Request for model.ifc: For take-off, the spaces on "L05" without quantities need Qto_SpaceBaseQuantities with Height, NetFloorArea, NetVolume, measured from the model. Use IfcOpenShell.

First a look at what the model holds.

```python
import ifcopenshell
import ifcopenshell.util.element
import ifcopenshell.util.unit

model = ifcopenshell.open("model.ifc")
print(model.schema)
for unit_type in ("LENGTHUNIT", "AREAUNIT", "VOLUMEUNIT"):
    print(unit_type, ifcopenshell.util.unit.calculate_unit_scale(model, unit_type))
storey = next(s for s in model.by_type("IfcBuildingStorey") if s.Name == "L05")
spaces = [e for e in ifcopenshell.util.element.get_decomposition(storey) if e.is_a("IfcSpace")]
for e in sorted(spaces, key=lambda e: e.id()):
    print(e.id(), e.is_a(), e.Name, list(ifcopenshell.util.element.get_psets(e, qtos_only=True)), sep=" | ")
```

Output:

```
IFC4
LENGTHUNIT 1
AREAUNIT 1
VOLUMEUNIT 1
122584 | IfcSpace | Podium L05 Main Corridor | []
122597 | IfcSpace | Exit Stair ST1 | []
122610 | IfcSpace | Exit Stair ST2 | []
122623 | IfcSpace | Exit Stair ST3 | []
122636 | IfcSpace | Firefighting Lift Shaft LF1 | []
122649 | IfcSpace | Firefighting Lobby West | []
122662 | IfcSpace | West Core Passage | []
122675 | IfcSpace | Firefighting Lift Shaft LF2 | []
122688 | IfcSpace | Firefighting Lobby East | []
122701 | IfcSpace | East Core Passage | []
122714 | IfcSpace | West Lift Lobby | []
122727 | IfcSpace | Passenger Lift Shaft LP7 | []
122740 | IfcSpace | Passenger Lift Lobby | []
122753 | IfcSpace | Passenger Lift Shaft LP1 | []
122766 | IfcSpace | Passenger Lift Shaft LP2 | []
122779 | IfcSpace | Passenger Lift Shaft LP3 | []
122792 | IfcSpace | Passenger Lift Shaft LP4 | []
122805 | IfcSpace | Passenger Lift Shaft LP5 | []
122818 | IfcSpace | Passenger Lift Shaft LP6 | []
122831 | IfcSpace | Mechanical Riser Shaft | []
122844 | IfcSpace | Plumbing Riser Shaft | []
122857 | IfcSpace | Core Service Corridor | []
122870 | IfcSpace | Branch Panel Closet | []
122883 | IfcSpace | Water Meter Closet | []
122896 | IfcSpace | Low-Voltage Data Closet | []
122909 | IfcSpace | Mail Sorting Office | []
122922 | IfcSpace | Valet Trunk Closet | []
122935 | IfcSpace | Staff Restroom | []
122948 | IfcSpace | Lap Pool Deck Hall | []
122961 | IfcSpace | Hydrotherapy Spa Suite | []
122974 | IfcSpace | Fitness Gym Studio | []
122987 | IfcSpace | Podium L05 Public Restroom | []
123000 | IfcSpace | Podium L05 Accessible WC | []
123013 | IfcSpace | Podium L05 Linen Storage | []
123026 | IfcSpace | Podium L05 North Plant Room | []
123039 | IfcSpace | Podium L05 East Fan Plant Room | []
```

```python
import ifcopenshell
import ifcopenshell.api.pset
import ifcopenshell.geom
import ifcopenshell.util.element
import ifcopenshell.util.shape
import ifcopenshell.util.unit

model = ifcopenshell.open("model.ifc")
unit_scale = ifcopenshell.util.unit.calculate_unit_scale(model)
area_scale = ifcopenshell.util.unit.calculate_unit_scale(model, "AREAUNIT")
volume_scale = ifcopenshell.util.unit.calculate_unit_scale(model, "VOLUMEUNIT")
settings = ifcopenshell.geom.settings()

storey = next(s for s in model.by_type("IfcBuildingStorey") if s.Name == "L05")
spaces = [e for e in ifcopenshell.util.element.get_decomposition(storey) if e.is_a("IfcSpace")]

for e in sorted(spaces, key=lambda e: e.id()):
    if ifcopenshell.util.element.get_psets(e, qtos_only=True, should_inherit=False):
        continue
    # Geometry comes back in metres, in the element's own axes.
    shape = ifcopenshell.geom.create_shape(settings, e)
    values = {
        "Height": ifcopenshell.util.shape.get_z(shape.geometry) / unit_scale,
        "NetFloorArea": ifcopenshell.util.shape.get_footprint_area(shape.geometry) / area_scale,
        "NetVolume": ifcopenshell.util.shape.get_volume(shape.geometry) / volume_scale,
    }
    qto = ifcopenshell.api.pset.add_qto(model, product=e, name="Qto_SpaceBaseQuantities")
    ifcopenshell.api.pset.edit_qto(model, qto=qto, properties=values)
    print(e.id(), {k: round(v, 3) for k, v in values.items()})

model.write("model_rev.ifc")
```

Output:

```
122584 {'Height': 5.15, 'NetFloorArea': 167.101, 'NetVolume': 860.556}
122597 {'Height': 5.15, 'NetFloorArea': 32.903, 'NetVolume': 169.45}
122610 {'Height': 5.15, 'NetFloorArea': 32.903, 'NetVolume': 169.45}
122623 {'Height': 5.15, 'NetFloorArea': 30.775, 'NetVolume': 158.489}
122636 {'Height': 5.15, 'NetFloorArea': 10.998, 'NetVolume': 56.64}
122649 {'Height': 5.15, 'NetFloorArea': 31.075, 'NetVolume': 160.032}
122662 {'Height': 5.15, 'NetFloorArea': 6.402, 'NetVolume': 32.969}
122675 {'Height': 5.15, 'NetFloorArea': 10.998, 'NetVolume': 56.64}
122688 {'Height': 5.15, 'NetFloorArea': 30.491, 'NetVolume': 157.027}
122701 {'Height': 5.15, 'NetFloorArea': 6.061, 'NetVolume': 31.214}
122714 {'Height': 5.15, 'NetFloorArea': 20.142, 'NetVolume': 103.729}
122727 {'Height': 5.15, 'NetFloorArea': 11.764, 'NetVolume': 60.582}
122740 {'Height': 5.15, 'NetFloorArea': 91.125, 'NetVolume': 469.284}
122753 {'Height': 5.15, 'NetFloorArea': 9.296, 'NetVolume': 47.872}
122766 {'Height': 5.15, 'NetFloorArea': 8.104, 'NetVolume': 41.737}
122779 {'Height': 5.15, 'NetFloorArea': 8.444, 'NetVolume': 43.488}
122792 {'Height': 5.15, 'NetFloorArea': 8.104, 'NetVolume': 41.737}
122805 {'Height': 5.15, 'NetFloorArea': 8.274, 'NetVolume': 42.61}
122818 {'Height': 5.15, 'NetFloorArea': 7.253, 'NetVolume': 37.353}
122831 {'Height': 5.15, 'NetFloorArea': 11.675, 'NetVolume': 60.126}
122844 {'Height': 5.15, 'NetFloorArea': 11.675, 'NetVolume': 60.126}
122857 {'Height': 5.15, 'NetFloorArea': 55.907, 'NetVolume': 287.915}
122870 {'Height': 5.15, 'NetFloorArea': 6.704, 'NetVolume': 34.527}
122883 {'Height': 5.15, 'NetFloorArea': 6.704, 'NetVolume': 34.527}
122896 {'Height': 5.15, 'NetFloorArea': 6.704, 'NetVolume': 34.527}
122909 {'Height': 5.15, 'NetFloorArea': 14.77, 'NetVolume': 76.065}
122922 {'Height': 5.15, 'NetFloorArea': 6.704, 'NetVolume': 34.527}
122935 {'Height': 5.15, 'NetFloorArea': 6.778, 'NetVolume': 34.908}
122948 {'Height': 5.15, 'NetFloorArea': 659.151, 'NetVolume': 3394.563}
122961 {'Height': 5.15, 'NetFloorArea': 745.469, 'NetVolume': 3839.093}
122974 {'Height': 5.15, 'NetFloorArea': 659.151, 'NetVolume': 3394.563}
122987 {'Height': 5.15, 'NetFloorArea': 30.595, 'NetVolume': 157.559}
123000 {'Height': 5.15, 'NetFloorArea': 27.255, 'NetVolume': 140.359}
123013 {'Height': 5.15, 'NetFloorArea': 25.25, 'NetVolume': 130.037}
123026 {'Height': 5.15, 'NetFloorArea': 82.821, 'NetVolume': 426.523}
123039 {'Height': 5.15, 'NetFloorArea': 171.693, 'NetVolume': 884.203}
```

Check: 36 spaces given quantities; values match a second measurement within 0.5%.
